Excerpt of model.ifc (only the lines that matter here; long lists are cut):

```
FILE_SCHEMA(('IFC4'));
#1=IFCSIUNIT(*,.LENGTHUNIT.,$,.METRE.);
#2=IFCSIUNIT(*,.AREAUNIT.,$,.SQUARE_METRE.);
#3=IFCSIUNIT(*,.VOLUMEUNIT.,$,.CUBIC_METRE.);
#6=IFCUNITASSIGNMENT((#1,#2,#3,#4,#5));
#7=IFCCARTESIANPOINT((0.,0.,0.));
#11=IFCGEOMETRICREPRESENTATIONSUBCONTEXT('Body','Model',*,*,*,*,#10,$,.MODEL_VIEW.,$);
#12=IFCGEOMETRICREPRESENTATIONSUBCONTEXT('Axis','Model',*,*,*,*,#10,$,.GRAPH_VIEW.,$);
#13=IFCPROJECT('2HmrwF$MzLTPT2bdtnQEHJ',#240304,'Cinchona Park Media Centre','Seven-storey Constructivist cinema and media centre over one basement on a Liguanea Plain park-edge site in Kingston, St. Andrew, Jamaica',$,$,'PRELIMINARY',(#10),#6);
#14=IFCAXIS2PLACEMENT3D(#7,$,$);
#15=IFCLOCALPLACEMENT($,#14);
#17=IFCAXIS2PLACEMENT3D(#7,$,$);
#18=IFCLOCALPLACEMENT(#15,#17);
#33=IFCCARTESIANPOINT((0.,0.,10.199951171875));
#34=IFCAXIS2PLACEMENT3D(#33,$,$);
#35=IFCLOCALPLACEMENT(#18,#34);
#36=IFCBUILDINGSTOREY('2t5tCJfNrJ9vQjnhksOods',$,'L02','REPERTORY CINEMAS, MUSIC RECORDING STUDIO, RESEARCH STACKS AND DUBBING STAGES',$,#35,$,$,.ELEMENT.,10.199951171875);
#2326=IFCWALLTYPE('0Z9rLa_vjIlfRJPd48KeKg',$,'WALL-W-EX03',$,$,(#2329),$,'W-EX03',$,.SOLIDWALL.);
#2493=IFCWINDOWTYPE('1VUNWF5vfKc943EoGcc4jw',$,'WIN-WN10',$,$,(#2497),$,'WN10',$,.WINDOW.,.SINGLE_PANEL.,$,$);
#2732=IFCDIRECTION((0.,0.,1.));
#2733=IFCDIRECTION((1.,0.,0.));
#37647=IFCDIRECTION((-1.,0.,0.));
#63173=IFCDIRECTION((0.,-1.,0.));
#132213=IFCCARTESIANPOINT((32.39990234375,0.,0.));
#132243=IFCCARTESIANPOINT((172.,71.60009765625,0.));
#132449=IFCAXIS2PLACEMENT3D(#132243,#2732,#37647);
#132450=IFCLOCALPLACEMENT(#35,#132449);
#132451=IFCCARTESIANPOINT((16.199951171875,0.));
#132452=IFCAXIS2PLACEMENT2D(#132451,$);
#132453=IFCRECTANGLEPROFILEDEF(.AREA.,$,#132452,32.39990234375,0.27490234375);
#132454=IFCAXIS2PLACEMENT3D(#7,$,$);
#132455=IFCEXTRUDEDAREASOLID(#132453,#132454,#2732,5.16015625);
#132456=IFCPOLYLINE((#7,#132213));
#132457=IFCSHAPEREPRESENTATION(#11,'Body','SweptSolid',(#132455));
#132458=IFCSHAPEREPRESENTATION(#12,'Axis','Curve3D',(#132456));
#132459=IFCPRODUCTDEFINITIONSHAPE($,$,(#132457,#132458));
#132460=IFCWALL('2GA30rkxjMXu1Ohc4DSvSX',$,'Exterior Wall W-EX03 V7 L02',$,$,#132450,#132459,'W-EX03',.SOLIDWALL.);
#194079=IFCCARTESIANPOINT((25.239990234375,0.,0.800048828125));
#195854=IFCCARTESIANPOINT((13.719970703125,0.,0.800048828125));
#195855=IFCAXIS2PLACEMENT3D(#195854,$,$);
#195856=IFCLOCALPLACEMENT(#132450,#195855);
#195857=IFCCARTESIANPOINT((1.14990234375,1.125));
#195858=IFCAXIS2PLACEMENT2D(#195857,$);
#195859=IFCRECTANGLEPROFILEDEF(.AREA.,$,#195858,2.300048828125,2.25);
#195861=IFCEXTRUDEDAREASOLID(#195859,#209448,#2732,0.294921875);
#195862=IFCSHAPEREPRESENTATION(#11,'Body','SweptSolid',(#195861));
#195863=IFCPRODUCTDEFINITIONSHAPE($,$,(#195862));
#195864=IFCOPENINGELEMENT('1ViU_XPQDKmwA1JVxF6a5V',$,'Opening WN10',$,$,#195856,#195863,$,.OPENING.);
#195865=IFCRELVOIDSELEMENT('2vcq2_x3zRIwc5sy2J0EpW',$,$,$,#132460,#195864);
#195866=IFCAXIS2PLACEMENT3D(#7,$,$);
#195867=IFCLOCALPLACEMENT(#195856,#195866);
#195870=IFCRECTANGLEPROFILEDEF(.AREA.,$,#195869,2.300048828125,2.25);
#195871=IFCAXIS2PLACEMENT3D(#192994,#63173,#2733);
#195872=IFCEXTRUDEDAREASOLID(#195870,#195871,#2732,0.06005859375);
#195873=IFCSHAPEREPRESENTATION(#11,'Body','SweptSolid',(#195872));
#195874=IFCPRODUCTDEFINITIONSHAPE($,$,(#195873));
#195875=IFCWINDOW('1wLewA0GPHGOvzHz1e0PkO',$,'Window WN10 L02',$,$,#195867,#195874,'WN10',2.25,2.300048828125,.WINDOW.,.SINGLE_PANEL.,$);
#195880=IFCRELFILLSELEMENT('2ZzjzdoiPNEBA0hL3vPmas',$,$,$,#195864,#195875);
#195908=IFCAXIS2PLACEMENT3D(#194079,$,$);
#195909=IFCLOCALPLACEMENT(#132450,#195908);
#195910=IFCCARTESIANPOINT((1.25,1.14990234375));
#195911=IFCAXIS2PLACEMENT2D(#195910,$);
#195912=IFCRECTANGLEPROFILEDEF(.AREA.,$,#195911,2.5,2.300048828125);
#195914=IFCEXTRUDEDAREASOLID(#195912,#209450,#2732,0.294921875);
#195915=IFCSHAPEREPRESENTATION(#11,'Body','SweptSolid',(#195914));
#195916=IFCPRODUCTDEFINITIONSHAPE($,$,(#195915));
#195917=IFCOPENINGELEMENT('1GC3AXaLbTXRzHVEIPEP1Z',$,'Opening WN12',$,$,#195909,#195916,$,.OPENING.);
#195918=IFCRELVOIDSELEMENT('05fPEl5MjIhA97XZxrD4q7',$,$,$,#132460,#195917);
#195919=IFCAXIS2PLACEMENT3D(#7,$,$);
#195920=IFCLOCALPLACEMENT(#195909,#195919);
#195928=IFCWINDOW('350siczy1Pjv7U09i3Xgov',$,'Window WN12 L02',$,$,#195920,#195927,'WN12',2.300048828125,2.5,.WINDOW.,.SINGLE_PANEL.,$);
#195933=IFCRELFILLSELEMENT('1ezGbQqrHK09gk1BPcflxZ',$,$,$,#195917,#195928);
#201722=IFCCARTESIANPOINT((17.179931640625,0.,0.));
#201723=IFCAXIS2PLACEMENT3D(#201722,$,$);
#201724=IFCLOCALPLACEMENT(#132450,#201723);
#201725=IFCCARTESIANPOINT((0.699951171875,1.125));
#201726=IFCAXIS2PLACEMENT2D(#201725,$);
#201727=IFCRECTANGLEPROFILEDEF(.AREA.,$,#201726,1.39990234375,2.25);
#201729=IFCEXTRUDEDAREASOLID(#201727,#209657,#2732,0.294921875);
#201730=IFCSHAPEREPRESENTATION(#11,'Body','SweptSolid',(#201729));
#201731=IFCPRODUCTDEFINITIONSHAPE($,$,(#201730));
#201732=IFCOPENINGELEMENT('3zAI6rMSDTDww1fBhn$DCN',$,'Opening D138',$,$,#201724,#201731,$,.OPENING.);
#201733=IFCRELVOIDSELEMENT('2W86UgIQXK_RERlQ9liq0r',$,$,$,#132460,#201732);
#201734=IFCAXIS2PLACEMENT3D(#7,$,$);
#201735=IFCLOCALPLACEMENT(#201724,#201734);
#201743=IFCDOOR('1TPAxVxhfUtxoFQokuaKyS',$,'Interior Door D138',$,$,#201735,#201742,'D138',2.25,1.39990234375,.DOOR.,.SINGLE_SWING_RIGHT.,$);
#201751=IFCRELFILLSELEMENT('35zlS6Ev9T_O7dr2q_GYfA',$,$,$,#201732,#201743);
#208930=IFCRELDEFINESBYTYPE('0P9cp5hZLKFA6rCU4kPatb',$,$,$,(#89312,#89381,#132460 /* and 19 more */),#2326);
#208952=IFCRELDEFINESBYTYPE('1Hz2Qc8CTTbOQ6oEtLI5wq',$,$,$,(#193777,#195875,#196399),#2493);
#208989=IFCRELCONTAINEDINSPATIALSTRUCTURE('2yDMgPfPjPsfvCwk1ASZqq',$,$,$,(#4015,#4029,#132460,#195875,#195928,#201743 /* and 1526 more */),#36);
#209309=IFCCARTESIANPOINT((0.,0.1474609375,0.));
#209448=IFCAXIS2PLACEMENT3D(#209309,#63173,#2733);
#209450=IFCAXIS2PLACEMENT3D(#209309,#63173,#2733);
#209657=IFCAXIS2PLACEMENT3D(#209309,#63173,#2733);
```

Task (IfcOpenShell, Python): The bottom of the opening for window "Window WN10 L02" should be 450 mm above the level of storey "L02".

```python
import numpy as np
import ifcopenshell
import ifcopenshell.api.geometry
import ifcopenshell.geom
import ifcopenshell.util.element
import ifcopenshell.util.placement
import ifcopenshell.util.shape
import ifcopenshell.util.unit

model = ifcopenshell.open("model.ifc")
unit_scale = ifcopenshell.util.unit.calculate_unit_scale(model)

window = model.by_guid("1wLewA0GPHGOvzHz1e0PkO")
opening = window.FillsVoids[0].RelatingOpeningElement
storey = ifcopenshell.util.element.get_container(window, ifc_class="IfcBuildingStorey")
level = ifcopenshell.util.placement.get_local_placement(storey.ObjectPlacement)[2, 3]

# The opening's origin need not be at the sill, so measure its lowest point.
shape = ifcopenshell.geom.create_shape(ifcopenshell.geom.settings(), opening)
bottom = ifcopenshell.util.shape.get_shape_bottom_elevation(shape, shape.geometry) / unit_scale
dz = level + 0.45 - bottom

shift = np.array([0.0, 0.0, dz])
# The window is placed relative to its opening, so it follows when the opening moves.
matrix = ifcopenshell.util.placement.get_local_placement(opening.ObjectPlacement)
matrix[:3, 3] += shift
ifcopenshell.api.geometry.edit_object_placement(
    model, product=opening, matrix=matrix, is_si=False, should_transform_children=True
)

print(f"moved by {dz * unit_scale:+.3f} m")

model.write("model_v2.ifc")
```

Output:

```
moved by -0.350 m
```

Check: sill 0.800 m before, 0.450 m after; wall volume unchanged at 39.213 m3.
